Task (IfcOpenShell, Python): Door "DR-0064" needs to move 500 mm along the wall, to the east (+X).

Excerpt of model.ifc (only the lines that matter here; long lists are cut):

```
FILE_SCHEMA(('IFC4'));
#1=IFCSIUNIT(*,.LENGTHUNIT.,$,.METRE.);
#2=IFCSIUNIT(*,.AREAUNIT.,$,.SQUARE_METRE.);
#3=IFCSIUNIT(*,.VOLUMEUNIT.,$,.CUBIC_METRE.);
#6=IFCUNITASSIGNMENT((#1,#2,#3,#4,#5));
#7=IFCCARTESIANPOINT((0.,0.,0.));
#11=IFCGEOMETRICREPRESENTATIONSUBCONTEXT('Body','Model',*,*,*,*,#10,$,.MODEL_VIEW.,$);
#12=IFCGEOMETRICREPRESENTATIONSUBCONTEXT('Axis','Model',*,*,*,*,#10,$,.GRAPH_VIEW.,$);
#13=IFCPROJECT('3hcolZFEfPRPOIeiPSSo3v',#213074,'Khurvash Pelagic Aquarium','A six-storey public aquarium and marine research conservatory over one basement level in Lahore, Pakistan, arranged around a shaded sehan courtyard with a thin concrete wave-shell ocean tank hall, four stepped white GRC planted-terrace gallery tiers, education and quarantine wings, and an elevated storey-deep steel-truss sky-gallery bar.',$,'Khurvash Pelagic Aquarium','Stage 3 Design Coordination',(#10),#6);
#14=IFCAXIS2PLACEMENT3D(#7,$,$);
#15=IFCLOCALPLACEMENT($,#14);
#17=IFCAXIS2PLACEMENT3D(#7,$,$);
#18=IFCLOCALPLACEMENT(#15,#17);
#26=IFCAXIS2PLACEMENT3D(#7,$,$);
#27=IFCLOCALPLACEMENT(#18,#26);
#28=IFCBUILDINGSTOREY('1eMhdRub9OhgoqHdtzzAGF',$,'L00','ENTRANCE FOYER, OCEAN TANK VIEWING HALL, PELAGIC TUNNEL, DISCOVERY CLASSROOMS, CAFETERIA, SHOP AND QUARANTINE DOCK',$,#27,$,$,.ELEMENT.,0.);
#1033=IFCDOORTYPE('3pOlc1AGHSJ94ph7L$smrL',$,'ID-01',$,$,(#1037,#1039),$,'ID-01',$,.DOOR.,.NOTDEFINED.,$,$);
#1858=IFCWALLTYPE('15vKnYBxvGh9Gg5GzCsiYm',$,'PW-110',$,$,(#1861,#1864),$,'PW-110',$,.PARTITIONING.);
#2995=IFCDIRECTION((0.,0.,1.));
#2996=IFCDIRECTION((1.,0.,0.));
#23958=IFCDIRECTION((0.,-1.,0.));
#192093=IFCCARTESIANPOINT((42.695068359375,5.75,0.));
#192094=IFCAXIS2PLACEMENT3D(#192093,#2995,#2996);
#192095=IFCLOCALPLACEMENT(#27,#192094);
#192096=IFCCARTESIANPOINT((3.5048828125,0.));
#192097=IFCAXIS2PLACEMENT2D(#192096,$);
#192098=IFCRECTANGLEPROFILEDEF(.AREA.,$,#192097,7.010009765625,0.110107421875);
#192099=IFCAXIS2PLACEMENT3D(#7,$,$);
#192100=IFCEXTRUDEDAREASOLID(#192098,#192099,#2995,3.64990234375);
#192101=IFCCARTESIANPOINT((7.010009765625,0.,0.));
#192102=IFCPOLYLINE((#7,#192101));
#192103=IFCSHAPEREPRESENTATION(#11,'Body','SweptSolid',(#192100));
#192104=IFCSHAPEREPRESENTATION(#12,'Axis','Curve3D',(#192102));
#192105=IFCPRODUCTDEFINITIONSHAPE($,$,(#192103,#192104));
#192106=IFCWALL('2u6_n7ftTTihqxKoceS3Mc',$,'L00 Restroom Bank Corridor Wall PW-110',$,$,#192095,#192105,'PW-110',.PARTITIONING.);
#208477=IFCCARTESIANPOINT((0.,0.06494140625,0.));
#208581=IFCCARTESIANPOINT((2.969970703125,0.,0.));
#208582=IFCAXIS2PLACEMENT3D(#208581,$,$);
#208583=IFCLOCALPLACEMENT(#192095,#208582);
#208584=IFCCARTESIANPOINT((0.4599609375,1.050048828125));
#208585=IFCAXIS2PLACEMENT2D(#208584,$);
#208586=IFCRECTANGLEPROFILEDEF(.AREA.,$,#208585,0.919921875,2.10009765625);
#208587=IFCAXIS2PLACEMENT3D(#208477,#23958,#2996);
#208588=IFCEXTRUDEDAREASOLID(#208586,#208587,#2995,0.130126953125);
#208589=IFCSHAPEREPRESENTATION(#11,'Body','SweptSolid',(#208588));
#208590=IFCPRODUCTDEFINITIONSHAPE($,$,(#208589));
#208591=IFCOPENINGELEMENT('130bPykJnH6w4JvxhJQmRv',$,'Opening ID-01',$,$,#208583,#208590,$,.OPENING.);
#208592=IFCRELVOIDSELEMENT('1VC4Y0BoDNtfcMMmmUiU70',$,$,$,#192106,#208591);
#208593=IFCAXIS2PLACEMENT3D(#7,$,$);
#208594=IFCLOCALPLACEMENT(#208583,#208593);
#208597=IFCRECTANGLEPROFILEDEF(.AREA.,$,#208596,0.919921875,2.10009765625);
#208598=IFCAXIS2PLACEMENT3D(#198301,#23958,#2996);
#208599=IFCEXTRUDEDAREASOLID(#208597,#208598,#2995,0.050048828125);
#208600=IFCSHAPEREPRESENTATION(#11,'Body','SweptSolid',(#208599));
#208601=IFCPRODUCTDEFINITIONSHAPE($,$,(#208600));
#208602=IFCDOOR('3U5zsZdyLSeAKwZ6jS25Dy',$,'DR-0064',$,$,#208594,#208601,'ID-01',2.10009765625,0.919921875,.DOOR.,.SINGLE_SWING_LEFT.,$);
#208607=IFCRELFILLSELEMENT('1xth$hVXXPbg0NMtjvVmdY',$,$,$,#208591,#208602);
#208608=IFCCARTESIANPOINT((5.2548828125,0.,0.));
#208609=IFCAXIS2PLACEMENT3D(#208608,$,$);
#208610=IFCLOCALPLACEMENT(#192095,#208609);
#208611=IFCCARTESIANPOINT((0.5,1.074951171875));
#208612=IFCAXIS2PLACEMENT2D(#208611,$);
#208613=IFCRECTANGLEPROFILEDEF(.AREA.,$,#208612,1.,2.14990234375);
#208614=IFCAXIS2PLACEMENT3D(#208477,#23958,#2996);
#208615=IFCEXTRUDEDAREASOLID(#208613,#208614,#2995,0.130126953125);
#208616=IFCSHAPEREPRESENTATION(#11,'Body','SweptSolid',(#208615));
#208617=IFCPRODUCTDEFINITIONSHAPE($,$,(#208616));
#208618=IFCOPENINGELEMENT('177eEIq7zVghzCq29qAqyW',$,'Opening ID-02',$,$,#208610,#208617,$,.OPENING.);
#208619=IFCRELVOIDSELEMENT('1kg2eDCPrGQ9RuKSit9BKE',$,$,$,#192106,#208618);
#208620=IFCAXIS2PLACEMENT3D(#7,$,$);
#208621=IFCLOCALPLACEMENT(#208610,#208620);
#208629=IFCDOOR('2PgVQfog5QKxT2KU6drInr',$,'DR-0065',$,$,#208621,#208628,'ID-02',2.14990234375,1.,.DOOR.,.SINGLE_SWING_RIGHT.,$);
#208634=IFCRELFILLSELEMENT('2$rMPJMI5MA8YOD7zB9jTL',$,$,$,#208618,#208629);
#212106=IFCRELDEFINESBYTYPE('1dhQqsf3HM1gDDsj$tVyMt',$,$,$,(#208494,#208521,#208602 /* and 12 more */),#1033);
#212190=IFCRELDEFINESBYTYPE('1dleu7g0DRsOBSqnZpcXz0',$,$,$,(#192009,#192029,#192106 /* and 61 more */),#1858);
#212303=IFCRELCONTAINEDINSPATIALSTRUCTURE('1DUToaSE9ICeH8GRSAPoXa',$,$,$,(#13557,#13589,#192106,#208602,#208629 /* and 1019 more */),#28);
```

```python
import ifcopenshell
import ifcopenshell.api.geometry
import ifcopenshell.util.placement
import ifcopenshell.util.unit

model = ifcopenshell.open("model.ifc")
unit_scale = ifcopenshell.util.unit.calculate_unit_scale(model)

door = model.by_guid("3U5zsZdyLSeAKwZ6jS25Dy")
opening = door.FillsVoids[0].RelatingOpeningElement
wall = opening.VoidsElements[0].RelatingBuildingElement

wall_matrix = ifcopenshell.util.placement.get_local_placement(wall.ObjectPlacement)
shift = wall_matrix[:3, 0] * 0.5 / unit_scale
before = ifcopenshell.util.placement.get_local_placement(door.ObjectPlacement)[:3, 3].copy()

# The door is placed relative to its opening, so it follows when the opening moves.
matrix = ifcopenshell.util.placement.get_local_placement(opening.ObjectPlacement)
matrix[:3, 3] += shift
ifcopenshell.api.geometry.edit_object_placement(
    model, product=opening, matrix=matrix, is_si=False, should_transform_children=True
)

after = ifcopenshell.util.placement.get_local_placement(door.ObjectPlacement)[:3, 3]
print("door moved by", (after - before).round(3) + 0.0)

model.write("model_v2.ifc")
```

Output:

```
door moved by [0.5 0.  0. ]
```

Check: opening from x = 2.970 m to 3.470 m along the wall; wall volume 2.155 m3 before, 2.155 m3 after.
